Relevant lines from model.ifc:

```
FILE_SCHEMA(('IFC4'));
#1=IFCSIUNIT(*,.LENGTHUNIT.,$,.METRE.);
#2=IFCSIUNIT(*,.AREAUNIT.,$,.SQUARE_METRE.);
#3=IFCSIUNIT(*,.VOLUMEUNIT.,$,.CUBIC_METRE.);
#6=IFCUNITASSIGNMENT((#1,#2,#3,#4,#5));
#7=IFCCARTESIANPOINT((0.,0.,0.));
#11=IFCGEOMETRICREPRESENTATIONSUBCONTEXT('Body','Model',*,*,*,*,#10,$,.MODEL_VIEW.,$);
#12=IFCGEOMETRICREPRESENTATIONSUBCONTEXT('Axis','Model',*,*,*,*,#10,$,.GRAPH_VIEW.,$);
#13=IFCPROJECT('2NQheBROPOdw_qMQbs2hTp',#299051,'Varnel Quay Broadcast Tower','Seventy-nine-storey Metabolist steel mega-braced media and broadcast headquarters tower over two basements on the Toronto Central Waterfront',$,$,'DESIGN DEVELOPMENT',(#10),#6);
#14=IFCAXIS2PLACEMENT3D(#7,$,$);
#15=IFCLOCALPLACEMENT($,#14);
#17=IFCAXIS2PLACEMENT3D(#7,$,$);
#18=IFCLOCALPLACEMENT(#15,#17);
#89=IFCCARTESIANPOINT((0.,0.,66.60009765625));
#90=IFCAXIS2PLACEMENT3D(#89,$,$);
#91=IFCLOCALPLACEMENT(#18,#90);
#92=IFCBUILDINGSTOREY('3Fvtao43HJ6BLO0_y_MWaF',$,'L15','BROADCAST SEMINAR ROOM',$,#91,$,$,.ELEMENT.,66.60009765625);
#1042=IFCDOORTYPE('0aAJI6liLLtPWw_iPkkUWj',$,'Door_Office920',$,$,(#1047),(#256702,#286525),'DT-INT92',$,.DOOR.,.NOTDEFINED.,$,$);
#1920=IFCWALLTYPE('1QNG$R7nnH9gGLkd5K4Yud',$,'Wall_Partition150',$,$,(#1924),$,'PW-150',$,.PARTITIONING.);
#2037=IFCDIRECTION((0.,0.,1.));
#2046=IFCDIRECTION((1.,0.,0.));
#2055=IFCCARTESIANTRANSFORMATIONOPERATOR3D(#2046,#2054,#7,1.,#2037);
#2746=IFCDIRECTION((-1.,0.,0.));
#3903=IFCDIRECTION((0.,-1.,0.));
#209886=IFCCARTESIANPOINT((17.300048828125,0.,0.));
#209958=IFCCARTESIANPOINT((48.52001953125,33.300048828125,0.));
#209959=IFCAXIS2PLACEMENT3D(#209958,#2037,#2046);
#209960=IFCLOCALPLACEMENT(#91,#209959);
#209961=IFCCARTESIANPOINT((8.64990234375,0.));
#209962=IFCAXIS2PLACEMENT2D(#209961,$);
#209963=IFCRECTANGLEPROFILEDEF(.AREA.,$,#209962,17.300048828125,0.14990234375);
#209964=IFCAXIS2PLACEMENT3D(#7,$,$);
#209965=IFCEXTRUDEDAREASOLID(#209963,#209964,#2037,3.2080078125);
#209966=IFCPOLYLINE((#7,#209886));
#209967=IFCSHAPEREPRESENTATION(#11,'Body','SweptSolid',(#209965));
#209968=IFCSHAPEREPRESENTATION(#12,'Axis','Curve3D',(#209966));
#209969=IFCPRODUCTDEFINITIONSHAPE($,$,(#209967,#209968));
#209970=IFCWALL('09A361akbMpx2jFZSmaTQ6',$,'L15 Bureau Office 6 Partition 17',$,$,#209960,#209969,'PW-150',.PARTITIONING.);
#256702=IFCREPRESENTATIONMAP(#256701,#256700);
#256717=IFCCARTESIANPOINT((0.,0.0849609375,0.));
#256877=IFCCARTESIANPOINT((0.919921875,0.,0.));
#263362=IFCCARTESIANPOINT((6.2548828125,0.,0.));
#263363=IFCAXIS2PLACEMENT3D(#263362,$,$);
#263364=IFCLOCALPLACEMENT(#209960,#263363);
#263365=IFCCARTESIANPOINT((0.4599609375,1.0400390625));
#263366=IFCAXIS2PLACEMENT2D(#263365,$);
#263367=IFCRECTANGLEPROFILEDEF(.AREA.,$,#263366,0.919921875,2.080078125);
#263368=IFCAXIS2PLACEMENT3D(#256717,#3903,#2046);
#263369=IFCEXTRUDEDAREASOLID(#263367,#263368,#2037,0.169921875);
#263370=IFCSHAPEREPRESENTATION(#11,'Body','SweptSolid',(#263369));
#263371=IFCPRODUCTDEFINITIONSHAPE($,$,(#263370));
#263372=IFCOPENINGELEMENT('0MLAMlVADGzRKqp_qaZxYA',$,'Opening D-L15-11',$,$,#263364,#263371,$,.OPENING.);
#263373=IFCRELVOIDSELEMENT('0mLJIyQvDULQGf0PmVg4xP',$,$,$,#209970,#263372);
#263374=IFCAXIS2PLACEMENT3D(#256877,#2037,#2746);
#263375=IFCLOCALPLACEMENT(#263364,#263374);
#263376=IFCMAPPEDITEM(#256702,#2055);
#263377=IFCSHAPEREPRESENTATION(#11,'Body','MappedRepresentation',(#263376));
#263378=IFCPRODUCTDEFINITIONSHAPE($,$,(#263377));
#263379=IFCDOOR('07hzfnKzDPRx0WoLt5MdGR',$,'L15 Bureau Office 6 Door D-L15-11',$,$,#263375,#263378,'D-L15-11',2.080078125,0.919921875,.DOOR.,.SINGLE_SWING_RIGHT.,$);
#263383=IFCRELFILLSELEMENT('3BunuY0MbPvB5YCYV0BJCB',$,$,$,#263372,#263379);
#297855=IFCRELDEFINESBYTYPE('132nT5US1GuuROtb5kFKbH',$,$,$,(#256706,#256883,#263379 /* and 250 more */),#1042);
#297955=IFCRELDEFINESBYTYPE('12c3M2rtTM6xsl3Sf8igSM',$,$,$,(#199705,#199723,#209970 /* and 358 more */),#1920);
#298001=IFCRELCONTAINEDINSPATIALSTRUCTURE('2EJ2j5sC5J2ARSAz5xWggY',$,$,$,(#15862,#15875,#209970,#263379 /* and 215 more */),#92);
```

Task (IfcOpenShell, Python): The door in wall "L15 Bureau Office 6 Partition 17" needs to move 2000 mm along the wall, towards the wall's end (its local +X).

```python
import ifcopenshell
import ifcopenshell.api.geometry
import ifcopenshell.util.placement

model = ifcopenshell.open("model.ifc")

door = model.by_guid("07hzfnKzDPRx0WoLt5MdGR")
opening = door.FillsVoids[0].RelatingOpeningElement
wall = opening.VoidsElements[0].RelatingBuildingElement

wall_matrix = ifcopenshell.util.placement.get_local_placement(wall.ObjectPlacement)
shift = wall_matrix[:3, 0] * 2.0
before = ifcopenshell.util.placement.get_local_placement(door.ObjectPlacement)[:3, 3].copy()

# The door is placed relative to its opening, so it follows when the opening moves.
matrix = ifcopenshell.util.placement.get_local_placement(opening.ObjectPlacement)
matrix[:3, 3] += shift
ifcopenshell.api.geometry.edit_object_placement(
    model, product=opening, matrix=matrix, is_si=False, should_transform_children=True
)

after = ifcopenshell.util.placement.get_local_placement(door.ObjectPlacement)[:3, 3]
print("door moved by", (after - before).round(3) + 0.0)

model.write("model-out.ifc")
```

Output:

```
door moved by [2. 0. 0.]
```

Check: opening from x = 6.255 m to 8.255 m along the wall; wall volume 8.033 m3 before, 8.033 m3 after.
